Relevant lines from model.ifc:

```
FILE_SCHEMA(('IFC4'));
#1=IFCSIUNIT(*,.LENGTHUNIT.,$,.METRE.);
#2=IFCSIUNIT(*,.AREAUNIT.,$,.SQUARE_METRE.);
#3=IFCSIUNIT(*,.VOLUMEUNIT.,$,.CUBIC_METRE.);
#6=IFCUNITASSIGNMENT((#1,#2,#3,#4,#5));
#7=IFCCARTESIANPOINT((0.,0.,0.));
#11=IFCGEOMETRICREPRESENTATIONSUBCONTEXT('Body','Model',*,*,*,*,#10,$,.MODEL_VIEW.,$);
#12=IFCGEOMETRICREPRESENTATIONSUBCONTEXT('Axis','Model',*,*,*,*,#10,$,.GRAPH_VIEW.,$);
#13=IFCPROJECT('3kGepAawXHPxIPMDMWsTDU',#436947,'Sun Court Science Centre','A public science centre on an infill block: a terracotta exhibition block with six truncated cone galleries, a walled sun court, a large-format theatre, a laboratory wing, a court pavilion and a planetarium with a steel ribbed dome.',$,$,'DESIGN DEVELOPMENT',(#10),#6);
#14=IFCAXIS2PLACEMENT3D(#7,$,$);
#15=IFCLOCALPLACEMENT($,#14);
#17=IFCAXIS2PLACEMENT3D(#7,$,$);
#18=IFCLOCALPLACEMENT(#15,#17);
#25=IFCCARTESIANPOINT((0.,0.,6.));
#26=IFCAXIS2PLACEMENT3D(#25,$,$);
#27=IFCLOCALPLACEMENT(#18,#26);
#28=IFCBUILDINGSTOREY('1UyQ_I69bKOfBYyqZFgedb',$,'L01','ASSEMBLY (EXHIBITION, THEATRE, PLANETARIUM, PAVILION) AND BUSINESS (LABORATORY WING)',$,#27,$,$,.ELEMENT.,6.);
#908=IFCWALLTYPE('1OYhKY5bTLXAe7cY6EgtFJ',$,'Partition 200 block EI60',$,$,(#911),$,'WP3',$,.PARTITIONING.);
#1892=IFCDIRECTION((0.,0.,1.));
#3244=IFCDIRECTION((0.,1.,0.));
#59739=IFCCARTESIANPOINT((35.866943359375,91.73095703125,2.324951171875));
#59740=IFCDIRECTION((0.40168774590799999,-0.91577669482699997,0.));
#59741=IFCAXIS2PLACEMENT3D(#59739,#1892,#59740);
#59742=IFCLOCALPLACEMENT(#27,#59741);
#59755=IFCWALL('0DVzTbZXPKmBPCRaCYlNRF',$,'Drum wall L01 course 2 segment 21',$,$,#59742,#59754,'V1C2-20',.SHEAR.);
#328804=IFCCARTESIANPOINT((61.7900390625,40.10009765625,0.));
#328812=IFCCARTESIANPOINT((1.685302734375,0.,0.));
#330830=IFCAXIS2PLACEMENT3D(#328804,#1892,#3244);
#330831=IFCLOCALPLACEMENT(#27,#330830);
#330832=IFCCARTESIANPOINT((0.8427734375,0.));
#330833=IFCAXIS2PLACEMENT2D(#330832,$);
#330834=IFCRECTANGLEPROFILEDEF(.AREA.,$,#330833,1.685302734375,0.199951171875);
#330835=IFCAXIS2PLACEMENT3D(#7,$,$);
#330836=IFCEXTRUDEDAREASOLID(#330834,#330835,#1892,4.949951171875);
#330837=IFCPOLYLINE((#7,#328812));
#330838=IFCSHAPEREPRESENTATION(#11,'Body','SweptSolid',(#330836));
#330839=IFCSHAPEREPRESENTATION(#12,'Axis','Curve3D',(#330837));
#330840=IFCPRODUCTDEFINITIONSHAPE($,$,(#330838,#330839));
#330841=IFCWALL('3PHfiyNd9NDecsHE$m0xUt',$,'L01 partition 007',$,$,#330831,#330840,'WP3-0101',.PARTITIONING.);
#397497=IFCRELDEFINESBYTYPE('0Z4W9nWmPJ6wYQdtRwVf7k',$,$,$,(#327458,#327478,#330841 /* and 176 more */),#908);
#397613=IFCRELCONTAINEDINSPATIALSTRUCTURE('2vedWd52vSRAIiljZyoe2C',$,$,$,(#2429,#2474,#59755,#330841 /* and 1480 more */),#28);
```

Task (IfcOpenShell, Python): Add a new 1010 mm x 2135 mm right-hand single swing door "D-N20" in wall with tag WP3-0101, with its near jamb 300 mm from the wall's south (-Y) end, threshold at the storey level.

```python
import numpy as np
import ifcopenshell
import ifcopenshell.api.feature
import ifcopenshell.api.geometry
import ifcopenshell.api.root
import ifcopenshell.api.spatial
import ifcopenshell.geom
import ifcopenshell.util.element
import ifcopenshell.util.placement
import ifcopenshell.util.representation
import ifcopenshell.util.shape
import ifcopenshell.util.unit

model = ifcopenshell.open("model.ifc")
unit_scale = ifcopenshell.util.unit.calculate_unit_scale(model)
settings = ifcopenshell.geom.settings()


def volume(element):
    """Net volume in cubic metres, openings subtracted."""
    shape = ifcopenshell.geom.create_shape(settings, element)
    return ifcopenshell.util.shape.get_volume(shape.geometry)


wall = model.by_guid("3PHfiyNd9NDecsHE$m0xUt")
storey = ifcopenshell.util.element.get_container(wall, ifc_class="IfcBuildingStorey")
context = ifcopenshell.util.representation.get_context(model, "Model", "Body", "MODEL_VIEW")
before = volume(wall)

width, height, from_end, sill = 1.01, 2.135, 0.3, 0.0  # metres

# The wall runs along its own X axis, and the end named is its -X end.
wall_shape = ifcopenshell.geom.create_shape(settings, wall)
x, y, z = ifcopenshell.util.shape.get_vertices(wall_shape.geometry).T
start = x.min() + from_end
face, thickness = float(y.min()), float(y.max() - y.min())
wall_matrix = ifcopenshell.util.placement.get_local_placement(wall.ObjectPlacement)
level = ifcopenshell.util.placement.get_local_placement(storey.ObjectPlacement)[2, 3]


def in_wall(x, y):
    """Placement at x, y metres in the wall's axes, at sill height."""
    matrix = wall_matrix.copy()
    matrix[:, 3] = wall_matrix @ np.array([x / unit_scale, y / unit_scale, 0.0, 1.0])
    matrix[2, 3] = level + sill / unit_scale
    return matrix


# Opening: a box that overshoots both wall faces by 50 mm.
opening = ifcopenshell.api.root.create_entity(model, ifc_class="IfcOpeningElement", predefined_type="OPENING")
box = ifcopenshell.api.geometry.add_wall_representation(
    model, context=context, length=width, height=height, thickness=thickness + 0.1
)
ifcopenshell.api.geometry.assign_representation(model, product=opening, representation=box)
ifcopenshell.api.geometry.edit_object_placement(model, product=opening, matrix=in_wall(start, face - 0.05), is_si=False)
ifcopenshell.api.feature.add_feature(model, feature=opening, element=wall)

door = ifcopenshell.api.root.create_entity(model, ifc_class="IfcDoor", name="D-N20", predefined_type="DOOR")
door.OverallWidth, door.OverallHeight = width / unit_scale, height / unit_scale
door.OperationType = "SINGLE_SWING_RIGHT"
body = ifcopenshell.api.geometry.add_door_representation(
    model,
    context=context,
    overall_width=door.OverallWidth,
    overall_height=door.OverallHeight,
    operation_type="SINGLE_SWING_RIGHT",
    lining_properties={"LiningDepth": thickness / unit_scale, "ThresholdDepth": thickness / unit_scale},
)
ifcopenshell.api.geometry.assign_representation(model, product=door, representation=body)
ifcopenshell.api.spatial.assign_container(model, products=[door], relating_structure=storey)
ifcopenshell.api.feature.add_filling(model, opening=opening, element=door)

# The lining spans the wall, so the door starts at the wall face.
ifcopenshell.api.geometry.edit_object_placement(model, product=door, matrix=in_wall(start, face), is_si=False)

after = volume(wall)

print(f"wall volume {before:.3f} -> {after:.3f} m3")

model.write("model_v2.ifc")
```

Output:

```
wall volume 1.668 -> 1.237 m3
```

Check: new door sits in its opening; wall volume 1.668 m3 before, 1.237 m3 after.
